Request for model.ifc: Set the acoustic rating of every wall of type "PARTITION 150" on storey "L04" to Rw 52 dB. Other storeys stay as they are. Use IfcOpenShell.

First a look at what the model holds.

```python
import ifcopenshell
import ifcopenshell.util.element

model = ifcopenshell.open("model.ifc")
print(model.schema)
storey = next(s for s in model.by_type("IfcBuildingStorey") if s.Name == "L04")
walls = [e for e in ifcopenshell.util.element.get_decomposition(storey) if e.is_a("IfcWall")]
seen = {}
for e in walls:
    element_type = ifcopenshell.util.element.get_type(e)
    key = (element_type.Name if element_type != e and element_type else None, ifcopenshell.util.element.get_pset(e, "Pset_WallCommon", "AcousticRating"))
    seen[key] = seen.get(key, 0) + 1
for (name, value), count in sorted(seen.items(), key=str):
    print(count, "x", name, "|", value)
```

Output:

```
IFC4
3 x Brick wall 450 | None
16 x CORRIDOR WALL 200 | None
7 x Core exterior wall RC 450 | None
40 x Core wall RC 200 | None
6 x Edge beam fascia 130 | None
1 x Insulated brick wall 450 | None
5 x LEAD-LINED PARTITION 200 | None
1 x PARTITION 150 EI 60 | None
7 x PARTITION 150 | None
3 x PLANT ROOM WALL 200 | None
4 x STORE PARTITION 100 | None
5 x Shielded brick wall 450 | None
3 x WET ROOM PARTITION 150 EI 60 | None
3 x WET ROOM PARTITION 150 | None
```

```python
import ifcopenshell
import ifcopenshell.api.pset
import ifcopenshell.util.element

model = ifcopenshell.open("model.ifc")

storey = next(s for s in model.by_type("IfcBuildingStorey") if s.Name == "L04")
walls = [e for e in ifcopenshell.util.element.get_decomposition(storey) if e.is_a("IfcWall")]

count = 0
for e in walls:
    element_type = ifcopenshell.util.element.get_type(e)
    if element_type in (None, e) or element_type.Name != "PARTITION 150":
        continue
    # add_pset returns the element's existing set when there is one.
    pset = ifcopenshell.api.pset.add_pset(model, product=e, name="Pset_WallCommon")
    ifcopenshell.api.pset.edit_pset(model, pset=pset, properties={"AcousticRating": "Rw 52 dB"})
    count += 1

print(count, "walls updated")

model.write("model_updated.ifc")
```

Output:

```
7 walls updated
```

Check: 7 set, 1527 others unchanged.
